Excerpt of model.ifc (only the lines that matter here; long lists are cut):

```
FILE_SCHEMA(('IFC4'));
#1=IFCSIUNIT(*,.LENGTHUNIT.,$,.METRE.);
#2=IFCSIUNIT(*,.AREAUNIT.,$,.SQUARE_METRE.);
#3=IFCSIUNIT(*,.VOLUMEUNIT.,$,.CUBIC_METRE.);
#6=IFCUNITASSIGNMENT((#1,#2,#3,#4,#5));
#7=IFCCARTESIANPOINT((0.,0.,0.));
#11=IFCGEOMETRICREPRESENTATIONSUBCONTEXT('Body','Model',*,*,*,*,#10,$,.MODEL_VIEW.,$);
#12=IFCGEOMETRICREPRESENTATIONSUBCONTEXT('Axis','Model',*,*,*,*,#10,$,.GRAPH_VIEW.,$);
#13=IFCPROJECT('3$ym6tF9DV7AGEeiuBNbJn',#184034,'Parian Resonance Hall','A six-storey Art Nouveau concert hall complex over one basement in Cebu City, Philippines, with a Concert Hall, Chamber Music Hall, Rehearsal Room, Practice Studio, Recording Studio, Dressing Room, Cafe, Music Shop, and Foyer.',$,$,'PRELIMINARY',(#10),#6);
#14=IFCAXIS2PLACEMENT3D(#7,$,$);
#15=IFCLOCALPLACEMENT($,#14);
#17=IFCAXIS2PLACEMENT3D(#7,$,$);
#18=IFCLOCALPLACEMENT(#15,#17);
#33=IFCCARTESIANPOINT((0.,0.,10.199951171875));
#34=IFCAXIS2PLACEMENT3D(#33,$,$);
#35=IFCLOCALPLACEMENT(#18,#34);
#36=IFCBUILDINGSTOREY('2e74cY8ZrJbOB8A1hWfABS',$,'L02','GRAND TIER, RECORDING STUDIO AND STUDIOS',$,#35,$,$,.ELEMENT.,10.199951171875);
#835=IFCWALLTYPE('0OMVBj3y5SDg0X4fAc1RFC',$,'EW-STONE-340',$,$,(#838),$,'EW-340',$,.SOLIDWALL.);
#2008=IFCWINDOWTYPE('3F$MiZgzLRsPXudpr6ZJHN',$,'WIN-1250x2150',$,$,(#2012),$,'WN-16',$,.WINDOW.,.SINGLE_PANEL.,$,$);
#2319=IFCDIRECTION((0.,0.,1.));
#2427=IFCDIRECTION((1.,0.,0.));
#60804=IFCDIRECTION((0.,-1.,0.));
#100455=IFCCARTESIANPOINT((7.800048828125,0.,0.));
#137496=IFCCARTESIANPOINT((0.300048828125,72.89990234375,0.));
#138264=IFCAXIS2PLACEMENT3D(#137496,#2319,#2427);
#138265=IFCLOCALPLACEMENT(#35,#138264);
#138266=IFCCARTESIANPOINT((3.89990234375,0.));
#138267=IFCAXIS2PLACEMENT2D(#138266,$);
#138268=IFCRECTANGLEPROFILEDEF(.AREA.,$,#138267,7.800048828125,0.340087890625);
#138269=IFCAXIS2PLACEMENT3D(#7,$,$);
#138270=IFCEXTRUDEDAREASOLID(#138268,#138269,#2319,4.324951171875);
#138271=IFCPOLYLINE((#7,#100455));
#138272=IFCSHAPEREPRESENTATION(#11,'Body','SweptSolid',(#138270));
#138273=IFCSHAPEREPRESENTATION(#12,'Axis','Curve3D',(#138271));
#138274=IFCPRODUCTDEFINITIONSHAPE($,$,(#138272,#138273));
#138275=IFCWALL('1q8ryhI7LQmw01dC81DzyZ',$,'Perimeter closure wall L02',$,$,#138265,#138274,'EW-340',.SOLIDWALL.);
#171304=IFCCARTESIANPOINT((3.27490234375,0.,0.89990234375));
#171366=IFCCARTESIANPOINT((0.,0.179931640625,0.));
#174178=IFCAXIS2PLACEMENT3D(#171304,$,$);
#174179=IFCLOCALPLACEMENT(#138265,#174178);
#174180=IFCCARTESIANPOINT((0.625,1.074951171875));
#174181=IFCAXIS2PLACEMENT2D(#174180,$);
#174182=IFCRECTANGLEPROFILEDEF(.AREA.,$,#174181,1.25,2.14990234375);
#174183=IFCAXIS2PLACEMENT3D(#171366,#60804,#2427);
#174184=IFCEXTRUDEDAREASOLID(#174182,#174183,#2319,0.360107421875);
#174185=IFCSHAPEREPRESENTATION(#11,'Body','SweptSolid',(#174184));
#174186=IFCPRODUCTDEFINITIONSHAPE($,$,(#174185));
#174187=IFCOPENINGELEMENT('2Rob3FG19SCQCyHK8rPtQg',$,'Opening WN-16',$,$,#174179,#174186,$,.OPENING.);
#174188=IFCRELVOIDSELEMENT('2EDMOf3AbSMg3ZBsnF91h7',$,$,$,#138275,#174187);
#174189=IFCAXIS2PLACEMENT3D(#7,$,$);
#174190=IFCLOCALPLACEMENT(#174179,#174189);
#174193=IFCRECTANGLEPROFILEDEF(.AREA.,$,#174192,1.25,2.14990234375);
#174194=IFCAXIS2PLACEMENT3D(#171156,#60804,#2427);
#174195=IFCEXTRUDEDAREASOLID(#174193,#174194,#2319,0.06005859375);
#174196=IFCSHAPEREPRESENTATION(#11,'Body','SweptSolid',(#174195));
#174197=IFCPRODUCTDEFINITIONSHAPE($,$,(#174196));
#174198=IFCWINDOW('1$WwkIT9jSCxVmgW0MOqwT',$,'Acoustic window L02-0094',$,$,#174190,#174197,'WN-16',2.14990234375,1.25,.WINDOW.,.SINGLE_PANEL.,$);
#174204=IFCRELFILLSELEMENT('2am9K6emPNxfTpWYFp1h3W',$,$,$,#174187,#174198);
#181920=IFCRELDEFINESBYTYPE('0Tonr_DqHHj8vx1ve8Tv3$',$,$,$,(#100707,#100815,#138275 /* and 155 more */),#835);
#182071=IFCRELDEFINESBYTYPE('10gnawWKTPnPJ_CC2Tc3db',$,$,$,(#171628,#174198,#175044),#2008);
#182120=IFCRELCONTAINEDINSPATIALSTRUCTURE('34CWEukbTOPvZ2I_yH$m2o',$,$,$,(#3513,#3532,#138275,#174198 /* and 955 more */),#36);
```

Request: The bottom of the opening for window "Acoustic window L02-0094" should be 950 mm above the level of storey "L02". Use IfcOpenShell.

```python
import numpy as np
import ifcopenshell
import ifcopenshell.api.geometry
import ifcopenshell.geom
import ifcopenshell.util.element
import ifcopenshell.util.placement
import ifcopenshell.util.shape
import ifcopenshell.util.unit

model = ifcopenshell.open("model.ifc")
unit_scale = ifcopenshell.util.unit.calculate_unit_scale(model)

window = model.by_guid("1$WwkIT9jSCxVmgW0MOqwT")
opening = window.FillsVoids[0].RelatingOpeningElement
storey = ifcopenshell.util.element.get_container(window, ifc_class="IfcBuildingStorey")
level = ifcopenshell.util.placement.get_local_placement(storey.ObjectPlacement)[2, 3]

# The opening's origin need not be at the sill, so measure its lowest point.
shape = ifcopenshell.geom.create_shape(ifcopenshell.geom.settings(), opening)
bottom = ifcopenshell.util.shape.get_shape_bottom_elevation(shape, shape.geometry) / unit_scale
dz = level + 0.95 / unit_scale - bottom

shift = np.array([0.0, 0.0, dz])
# The window is placed relative to its opening, so it follows when the opening moves.
matrix = ifcopenshell.util.placement.get_local_placement(opening.ObjectPlacement)
matrix[:3, 3] += shift
ifcopenshell.api.geometry.edit_object_placement(
    model, product=opening, matrix=matrix, is_si=False, should_transform_children=True
)

print(f"moved by {dz * unit_scale:+.3f} m")

model.write("model_updated.ifc")
```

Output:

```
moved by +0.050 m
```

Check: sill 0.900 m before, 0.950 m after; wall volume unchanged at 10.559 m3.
